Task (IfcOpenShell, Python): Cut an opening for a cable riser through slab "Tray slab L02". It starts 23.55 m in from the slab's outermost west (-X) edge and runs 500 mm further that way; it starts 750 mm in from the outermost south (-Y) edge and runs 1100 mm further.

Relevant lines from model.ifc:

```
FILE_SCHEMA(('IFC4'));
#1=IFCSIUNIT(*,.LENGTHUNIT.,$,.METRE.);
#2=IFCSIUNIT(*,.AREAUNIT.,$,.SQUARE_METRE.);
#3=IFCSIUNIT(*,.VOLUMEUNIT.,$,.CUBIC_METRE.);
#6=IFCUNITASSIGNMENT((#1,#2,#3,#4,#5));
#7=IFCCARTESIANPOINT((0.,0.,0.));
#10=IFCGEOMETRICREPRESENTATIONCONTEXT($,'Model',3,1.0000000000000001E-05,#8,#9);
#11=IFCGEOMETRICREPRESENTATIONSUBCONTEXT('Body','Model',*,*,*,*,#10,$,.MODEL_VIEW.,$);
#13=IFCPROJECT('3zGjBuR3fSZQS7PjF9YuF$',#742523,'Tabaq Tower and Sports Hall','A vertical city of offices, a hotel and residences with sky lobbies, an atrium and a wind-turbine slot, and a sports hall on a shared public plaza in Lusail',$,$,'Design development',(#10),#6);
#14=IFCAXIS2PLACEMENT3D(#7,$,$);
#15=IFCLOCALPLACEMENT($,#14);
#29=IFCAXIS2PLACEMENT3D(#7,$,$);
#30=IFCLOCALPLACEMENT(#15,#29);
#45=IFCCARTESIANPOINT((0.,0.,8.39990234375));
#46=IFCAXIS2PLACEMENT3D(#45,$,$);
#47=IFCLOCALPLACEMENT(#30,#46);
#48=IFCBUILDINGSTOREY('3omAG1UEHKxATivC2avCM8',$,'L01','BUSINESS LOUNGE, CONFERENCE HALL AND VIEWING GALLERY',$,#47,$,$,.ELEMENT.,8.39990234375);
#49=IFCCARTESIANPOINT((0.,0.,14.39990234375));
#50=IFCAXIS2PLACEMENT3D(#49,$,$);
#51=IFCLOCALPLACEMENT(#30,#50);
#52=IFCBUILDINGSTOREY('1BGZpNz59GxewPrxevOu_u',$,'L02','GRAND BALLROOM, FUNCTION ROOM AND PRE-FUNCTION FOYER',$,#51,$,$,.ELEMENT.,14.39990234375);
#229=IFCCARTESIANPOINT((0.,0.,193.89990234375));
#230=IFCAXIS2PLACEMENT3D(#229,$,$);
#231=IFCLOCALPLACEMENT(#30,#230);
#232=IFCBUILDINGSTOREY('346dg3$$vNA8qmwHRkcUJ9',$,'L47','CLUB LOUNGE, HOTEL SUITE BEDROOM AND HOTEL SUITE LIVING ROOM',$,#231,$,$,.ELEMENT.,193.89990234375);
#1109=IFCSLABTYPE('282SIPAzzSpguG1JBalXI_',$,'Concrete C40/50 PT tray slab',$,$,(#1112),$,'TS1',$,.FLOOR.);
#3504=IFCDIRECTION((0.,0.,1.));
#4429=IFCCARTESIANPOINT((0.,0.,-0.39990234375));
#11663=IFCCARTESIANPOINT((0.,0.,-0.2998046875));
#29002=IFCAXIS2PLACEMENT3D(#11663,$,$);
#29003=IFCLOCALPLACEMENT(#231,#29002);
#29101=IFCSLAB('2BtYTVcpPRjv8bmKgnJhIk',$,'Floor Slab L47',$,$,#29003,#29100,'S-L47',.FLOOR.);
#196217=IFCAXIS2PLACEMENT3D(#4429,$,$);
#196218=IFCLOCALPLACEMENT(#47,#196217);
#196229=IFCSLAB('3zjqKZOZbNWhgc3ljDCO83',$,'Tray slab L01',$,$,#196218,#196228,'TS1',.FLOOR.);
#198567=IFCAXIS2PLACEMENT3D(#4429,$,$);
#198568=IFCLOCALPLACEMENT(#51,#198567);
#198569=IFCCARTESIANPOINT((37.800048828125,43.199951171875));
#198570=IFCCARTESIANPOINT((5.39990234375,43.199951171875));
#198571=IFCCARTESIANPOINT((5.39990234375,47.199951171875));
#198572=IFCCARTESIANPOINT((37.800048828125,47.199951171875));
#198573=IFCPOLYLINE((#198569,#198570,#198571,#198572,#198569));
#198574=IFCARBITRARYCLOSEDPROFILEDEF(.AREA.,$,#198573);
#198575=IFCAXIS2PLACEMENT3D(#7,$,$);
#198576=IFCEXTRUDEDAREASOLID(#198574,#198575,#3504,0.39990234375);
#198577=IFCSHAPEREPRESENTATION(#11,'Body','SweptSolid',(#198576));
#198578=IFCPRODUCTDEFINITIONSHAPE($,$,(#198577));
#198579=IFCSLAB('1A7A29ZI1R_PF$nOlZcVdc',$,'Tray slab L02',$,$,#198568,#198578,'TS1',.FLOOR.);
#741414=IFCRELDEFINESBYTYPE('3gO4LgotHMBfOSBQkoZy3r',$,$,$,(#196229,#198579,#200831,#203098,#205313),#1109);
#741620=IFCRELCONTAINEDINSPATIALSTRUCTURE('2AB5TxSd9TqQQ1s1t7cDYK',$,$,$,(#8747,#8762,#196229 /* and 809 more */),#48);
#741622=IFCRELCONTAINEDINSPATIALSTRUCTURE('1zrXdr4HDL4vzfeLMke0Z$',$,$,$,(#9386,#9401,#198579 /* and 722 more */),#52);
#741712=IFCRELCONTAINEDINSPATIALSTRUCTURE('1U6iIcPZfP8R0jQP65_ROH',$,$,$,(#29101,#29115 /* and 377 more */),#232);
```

```python
import numpy as np
import ifcopenshell
import ifcopenshell.api.feature
import ifcopenshell.api.geometry
import ifcopenshell.api.root
import ifcopenshell.geom
import ifcopenshell.util.placement
import ifcopenshell.util.representation
import ifcopenshell.util.shape
import ifcopenshell.util.unit

model = ifcopenshell.open("model.ifc")
unit_scale = ifcopenshell.util.unit.calculate_unit_scale(model)
settings = ifcopenshell.geom.settings()


def volume(element):
    """Net volume in cubic metres, openings subtracted."""
    shape = ifcopenshell.geom.create_shape(settings, element)
    return ifcopenshell.util.shape.get_volume(shape.geometry)


slab = model.by_id(198579)
before = volume(slab)

# Extent in the slab's own axes, in metres. The edges named are its -X and -Y sides.
slab_shape = ifcopenshell.geom.create_shape(settings, slab)
vertices = ifcopenshell.util.shape.get_vertices(slab_shape.geometry)
x_min, y_min, bottom = vertices.min(axis=0)
top = vertices[:, 2].max()

opening = ifcopenshell.api.root.create_entity(model, ifc_class="IfcOpeningElement", name="Cable riser opening", predefined_type="OPENING")
context = ifcopenshell.util.representation.get_context(model, "Model", "Body", "MODEL_VIEW")
width, depth = 0.5, 1.1
outline = [(0.0, 0.0), (width, 0.0), (width, depth), (0.0, depth), (0.0, 0.0)]
# Overshoot both faces by 50 mm so the cut is clean.
shape = ifcopenshell.api.geometry.add_slab_representation(
    model, context=context, depth=top - bottom + 0.1, polyline=outline
)
ifcopenshell.api.geometry.assign_representation(model, product=opening, representation=shape)

matrix = ifcopenshell.util.placement.get_local_placement(slab.ObjectPlacement)
matrix[:, 3] = matrix @ np.append(np.array([x_min + 23.55, y_min + 0.75, bottom - 0.05]) / unit_scale, 1.0)
ifcopenshell.api.geometry.edit_object_placement(model, product=opening, matrix=matrix, is_si=False)
ifcopenshell.api.feature.add_feature(model, feature=opening, element=slab)

after = volume(slab)

print(f"slab volume {before:.3f} -> {after:.3f} m3")

model.write("model_updated.ifc")
```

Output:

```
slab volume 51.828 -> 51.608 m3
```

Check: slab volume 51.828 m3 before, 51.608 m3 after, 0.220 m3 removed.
